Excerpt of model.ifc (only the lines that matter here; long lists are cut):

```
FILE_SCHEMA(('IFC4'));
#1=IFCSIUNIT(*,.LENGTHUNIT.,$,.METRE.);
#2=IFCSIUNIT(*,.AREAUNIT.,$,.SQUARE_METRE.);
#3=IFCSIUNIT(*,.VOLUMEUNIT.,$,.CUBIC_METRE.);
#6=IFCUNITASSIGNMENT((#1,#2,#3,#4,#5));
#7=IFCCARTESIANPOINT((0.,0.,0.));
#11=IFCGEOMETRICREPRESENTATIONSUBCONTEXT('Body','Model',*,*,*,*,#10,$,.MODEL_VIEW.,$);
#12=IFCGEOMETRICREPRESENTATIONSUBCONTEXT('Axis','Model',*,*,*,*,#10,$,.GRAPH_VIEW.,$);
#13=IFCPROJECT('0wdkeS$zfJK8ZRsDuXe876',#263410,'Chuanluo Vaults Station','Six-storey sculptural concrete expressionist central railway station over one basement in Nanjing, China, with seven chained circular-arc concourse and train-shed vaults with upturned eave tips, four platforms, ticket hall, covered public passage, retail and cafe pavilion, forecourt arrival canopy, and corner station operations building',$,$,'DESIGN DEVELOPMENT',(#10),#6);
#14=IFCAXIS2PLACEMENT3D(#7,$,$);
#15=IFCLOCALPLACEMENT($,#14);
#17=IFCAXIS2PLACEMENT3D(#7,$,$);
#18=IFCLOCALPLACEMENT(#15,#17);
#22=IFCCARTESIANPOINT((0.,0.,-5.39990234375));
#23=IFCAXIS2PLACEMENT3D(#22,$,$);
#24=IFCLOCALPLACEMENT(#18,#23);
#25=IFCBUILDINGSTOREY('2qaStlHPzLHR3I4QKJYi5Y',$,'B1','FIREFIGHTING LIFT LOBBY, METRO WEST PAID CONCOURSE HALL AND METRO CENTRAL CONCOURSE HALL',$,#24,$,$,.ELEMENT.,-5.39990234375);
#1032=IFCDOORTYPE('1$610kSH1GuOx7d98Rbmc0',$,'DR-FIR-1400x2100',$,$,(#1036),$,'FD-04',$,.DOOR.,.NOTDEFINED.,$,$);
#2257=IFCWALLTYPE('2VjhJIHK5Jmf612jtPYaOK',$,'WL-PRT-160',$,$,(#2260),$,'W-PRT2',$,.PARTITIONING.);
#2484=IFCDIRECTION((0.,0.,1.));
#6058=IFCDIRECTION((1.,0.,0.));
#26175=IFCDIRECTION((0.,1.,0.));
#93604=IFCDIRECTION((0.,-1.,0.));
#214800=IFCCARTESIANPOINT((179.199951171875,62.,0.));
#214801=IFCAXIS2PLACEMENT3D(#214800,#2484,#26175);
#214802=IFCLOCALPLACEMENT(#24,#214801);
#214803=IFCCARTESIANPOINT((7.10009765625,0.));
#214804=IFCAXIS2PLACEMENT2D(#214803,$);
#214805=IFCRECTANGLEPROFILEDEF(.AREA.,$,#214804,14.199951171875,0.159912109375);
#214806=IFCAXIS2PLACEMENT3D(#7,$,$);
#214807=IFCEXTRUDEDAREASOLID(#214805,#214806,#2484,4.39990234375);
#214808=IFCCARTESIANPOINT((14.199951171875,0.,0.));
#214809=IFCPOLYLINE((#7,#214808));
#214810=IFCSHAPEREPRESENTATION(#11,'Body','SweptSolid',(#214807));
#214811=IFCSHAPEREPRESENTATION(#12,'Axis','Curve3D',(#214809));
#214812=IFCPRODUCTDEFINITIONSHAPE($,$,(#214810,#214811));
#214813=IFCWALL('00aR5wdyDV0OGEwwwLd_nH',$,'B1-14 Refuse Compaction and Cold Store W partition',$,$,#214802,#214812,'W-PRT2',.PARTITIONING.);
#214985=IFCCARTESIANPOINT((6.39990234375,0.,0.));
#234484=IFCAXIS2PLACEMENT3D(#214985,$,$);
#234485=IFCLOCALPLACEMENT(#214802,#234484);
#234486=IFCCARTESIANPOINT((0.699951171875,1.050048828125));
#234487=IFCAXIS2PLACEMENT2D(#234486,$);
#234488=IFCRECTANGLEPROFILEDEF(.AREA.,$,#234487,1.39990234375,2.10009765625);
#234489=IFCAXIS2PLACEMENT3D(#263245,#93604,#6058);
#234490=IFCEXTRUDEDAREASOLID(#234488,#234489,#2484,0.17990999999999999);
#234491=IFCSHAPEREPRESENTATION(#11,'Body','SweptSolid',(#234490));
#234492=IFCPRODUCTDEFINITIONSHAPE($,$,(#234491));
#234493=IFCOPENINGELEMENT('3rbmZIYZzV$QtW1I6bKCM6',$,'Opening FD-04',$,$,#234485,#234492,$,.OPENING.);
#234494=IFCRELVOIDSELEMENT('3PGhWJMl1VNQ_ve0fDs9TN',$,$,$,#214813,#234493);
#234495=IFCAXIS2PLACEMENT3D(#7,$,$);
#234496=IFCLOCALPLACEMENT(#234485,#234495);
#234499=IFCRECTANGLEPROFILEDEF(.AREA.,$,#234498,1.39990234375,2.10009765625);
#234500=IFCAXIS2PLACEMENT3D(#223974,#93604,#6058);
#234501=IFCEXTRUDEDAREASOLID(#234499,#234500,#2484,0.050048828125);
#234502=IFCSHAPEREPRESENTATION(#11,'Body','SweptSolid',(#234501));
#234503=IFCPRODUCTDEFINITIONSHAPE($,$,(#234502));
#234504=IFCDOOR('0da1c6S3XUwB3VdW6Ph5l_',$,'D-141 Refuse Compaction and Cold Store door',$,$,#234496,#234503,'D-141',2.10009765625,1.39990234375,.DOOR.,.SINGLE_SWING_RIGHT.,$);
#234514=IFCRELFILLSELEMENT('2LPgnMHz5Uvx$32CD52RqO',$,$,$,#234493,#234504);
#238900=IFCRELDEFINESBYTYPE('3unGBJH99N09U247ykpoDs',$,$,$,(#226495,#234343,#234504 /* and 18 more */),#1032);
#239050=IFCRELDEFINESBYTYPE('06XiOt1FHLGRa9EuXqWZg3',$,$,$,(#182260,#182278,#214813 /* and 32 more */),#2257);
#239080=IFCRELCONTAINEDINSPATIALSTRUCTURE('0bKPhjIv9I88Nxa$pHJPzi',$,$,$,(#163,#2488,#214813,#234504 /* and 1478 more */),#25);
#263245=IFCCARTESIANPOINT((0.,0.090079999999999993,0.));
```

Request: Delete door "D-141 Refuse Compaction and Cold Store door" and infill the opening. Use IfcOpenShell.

```python
import ifcopenshell
import ifcopenshell.api.feature
import ifcopenshell.api.root
import ifcopenshell.geom
import ifcopenshell.util.shape

model = ifcopenshell.open("model.ifc")
settings = ifcopenshell.geom.settings()


def volume(element):
    """Net volume in cubic metres, openings subtracted."""
    shape = ifcopenshell.geom.create_shape(settings, element)
    return ifcopenshell.util.shape.get_volume(shape.geometry)


door = model.by_guid("0da1c6S3XUwB3VdW6Ph5l_")
opening = door.FillsVoids[0].RelatingOpeningElement
wall = opening.VoidsElements[0].RelatingBuildingElement
before = volume(wall)

ifcopenshell.api.root.remove_product(model, product=door)
ifcopenshell.api.feature.remove_feature(model, feature=opening)

after = volume(wall)

print(f"wall volume {before:.3f} -> {after:.3f} m3")

model.write("model_edited.ifc")
```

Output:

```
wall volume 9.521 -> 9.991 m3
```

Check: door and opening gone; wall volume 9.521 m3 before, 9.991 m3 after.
